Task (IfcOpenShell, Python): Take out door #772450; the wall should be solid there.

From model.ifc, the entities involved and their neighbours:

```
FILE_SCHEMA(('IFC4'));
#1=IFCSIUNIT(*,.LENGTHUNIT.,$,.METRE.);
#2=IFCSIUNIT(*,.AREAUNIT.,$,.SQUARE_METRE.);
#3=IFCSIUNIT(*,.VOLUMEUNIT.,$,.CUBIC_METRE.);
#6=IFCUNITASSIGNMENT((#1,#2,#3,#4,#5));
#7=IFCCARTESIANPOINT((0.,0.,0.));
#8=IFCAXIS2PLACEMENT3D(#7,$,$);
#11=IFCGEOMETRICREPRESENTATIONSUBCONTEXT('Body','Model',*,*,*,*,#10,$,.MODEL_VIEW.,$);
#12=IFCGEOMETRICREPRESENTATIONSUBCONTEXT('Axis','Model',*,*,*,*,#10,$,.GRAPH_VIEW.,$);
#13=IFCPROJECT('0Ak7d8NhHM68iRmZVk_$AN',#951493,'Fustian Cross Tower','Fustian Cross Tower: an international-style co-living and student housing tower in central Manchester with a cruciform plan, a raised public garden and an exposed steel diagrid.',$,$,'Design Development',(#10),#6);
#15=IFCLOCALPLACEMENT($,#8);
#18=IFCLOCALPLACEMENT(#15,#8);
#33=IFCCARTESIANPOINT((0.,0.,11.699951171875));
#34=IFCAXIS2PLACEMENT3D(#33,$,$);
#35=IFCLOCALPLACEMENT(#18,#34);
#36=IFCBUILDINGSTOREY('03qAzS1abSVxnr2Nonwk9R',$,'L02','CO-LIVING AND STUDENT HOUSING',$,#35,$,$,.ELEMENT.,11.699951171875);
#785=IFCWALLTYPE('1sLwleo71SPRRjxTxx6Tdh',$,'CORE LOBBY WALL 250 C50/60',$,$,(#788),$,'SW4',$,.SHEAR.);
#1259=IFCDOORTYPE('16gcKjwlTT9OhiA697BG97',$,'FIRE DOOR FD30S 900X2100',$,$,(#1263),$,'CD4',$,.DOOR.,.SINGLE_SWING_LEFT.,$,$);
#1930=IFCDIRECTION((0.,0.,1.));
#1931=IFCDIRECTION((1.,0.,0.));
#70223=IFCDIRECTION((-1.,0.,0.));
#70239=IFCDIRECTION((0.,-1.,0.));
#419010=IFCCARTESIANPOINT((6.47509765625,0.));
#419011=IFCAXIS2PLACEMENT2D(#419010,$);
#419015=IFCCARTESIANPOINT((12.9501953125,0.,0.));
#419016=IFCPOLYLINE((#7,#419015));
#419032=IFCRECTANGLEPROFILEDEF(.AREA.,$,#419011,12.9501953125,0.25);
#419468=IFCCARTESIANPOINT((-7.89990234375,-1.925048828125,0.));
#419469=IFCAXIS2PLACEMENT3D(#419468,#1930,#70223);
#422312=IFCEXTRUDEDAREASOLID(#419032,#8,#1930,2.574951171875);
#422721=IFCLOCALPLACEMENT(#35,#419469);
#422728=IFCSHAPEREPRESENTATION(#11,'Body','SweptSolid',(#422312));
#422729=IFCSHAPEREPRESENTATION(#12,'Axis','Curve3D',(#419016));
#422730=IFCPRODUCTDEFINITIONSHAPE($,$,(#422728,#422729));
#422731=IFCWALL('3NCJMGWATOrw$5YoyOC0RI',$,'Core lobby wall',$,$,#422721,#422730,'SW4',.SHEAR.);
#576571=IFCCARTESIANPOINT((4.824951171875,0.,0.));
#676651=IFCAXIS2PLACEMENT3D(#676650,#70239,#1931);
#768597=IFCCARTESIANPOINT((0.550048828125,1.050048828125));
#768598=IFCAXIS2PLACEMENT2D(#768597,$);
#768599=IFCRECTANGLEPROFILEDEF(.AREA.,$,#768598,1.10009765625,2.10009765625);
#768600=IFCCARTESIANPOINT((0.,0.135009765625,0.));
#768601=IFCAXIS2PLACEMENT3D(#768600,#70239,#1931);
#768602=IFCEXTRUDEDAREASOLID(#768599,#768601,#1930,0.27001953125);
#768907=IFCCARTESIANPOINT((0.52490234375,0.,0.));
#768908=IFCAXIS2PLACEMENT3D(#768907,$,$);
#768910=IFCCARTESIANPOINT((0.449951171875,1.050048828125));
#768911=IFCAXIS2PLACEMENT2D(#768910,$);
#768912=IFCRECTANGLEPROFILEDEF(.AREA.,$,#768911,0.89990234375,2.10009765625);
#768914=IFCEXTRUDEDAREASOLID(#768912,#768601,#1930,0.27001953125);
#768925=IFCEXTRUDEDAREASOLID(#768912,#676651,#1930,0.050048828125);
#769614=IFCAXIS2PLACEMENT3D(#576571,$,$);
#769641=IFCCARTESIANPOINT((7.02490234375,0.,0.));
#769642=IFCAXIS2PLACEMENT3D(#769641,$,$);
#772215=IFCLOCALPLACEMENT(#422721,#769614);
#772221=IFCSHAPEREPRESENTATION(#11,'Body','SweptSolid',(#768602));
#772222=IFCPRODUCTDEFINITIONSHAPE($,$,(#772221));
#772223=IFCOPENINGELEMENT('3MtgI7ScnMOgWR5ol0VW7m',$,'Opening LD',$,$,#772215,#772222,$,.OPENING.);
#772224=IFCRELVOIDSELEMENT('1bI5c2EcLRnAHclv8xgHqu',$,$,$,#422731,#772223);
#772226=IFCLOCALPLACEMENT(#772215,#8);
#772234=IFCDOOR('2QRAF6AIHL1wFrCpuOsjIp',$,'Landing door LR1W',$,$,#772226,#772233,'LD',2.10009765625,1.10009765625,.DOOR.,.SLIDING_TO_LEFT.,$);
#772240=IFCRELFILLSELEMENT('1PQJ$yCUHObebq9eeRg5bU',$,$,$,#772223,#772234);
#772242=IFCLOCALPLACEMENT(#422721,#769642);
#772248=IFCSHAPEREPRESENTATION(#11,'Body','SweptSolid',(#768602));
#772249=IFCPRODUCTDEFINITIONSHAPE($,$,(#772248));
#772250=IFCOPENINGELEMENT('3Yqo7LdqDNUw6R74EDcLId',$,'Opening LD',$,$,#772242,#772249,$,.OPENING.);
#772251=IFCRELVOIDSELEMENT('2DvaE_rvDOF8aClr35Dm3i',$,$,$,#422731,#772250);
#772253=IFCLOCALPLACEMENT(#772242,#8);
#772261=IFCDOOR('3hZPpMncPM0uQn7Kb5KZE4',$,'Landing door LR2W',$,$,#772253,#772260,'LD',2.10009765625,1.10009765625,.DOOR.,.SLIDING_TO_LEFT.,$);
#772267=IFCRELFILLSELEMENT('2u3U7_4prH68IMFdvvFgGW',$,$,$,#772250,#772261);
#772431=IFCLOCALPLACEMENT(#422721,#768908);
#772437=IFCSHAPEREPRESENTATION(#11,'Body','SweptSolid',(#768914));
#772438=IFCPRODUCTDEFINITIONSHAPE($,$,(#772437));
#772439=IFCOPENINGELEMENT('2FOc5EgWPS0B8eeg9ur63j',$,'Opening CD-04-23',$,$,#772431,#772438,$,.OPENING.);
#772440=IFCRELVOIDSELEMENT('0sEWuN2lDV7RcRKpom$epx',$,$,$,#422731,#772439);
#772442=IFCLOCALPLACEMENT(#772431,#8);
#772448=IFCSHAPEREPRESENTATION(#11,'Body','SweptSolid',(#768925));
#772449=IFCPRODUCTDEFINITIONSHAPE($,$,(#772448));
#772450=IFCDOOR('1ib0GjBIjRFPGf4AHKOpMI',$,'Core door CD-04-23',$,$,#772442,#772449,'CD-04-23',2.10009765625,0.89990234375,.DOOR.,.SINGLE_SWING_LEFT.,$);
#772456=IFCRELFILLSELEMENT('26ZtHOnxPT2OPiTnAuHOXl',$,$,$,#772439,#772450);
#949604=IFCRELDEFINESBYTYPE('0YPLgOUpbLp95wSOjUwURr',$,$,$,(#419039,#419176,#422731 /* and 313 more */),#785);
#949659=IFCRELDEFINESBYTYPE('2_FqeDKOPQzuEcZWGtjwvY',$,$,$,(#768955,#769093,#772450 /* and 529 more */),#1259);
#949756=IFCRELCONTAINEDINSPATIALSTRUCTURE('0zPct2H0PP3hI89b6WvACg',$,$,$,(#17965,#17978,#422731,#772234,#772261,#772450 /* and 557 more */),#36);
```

```python
import ifcopenshell
import ifcopenshell.api.feature
import ifcopenshell.api.root
import ifcopenshell.geom
import ifcopenshell.util.shape

model = ifcopenshell.open("model.ifc")
settings = ifcopenshell.geom.settings()


def volume(element):
    """Net volume in cubic metres, openings subtracted."""
    shape = ifcopenshell.geom.create_shape(settings, element)
    return ifcopenshell.util.shape.get_volume(shape.geometry)


door = model.by_guid("1ib0GjBIjRFPGf4AHKOpMI")
opening = door.FillsVoids[0].RelatingOpeningElement
wall = opening.VoidsElements[0].RelatingBuildingElement
before = volume(wall)

ifcopenshell.api.root.remove_product(model, product=door)
ifcopenshell.api.feature.remove_feature(model, feature=opening)

after = volume(wall)

print(f"wall volume {before:.3f} -> {after:.3f} m3")

model.write("model_updated.ifc")
```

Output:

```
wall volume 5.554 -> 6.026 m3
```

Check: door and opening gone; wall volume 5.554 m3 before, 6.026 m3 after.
